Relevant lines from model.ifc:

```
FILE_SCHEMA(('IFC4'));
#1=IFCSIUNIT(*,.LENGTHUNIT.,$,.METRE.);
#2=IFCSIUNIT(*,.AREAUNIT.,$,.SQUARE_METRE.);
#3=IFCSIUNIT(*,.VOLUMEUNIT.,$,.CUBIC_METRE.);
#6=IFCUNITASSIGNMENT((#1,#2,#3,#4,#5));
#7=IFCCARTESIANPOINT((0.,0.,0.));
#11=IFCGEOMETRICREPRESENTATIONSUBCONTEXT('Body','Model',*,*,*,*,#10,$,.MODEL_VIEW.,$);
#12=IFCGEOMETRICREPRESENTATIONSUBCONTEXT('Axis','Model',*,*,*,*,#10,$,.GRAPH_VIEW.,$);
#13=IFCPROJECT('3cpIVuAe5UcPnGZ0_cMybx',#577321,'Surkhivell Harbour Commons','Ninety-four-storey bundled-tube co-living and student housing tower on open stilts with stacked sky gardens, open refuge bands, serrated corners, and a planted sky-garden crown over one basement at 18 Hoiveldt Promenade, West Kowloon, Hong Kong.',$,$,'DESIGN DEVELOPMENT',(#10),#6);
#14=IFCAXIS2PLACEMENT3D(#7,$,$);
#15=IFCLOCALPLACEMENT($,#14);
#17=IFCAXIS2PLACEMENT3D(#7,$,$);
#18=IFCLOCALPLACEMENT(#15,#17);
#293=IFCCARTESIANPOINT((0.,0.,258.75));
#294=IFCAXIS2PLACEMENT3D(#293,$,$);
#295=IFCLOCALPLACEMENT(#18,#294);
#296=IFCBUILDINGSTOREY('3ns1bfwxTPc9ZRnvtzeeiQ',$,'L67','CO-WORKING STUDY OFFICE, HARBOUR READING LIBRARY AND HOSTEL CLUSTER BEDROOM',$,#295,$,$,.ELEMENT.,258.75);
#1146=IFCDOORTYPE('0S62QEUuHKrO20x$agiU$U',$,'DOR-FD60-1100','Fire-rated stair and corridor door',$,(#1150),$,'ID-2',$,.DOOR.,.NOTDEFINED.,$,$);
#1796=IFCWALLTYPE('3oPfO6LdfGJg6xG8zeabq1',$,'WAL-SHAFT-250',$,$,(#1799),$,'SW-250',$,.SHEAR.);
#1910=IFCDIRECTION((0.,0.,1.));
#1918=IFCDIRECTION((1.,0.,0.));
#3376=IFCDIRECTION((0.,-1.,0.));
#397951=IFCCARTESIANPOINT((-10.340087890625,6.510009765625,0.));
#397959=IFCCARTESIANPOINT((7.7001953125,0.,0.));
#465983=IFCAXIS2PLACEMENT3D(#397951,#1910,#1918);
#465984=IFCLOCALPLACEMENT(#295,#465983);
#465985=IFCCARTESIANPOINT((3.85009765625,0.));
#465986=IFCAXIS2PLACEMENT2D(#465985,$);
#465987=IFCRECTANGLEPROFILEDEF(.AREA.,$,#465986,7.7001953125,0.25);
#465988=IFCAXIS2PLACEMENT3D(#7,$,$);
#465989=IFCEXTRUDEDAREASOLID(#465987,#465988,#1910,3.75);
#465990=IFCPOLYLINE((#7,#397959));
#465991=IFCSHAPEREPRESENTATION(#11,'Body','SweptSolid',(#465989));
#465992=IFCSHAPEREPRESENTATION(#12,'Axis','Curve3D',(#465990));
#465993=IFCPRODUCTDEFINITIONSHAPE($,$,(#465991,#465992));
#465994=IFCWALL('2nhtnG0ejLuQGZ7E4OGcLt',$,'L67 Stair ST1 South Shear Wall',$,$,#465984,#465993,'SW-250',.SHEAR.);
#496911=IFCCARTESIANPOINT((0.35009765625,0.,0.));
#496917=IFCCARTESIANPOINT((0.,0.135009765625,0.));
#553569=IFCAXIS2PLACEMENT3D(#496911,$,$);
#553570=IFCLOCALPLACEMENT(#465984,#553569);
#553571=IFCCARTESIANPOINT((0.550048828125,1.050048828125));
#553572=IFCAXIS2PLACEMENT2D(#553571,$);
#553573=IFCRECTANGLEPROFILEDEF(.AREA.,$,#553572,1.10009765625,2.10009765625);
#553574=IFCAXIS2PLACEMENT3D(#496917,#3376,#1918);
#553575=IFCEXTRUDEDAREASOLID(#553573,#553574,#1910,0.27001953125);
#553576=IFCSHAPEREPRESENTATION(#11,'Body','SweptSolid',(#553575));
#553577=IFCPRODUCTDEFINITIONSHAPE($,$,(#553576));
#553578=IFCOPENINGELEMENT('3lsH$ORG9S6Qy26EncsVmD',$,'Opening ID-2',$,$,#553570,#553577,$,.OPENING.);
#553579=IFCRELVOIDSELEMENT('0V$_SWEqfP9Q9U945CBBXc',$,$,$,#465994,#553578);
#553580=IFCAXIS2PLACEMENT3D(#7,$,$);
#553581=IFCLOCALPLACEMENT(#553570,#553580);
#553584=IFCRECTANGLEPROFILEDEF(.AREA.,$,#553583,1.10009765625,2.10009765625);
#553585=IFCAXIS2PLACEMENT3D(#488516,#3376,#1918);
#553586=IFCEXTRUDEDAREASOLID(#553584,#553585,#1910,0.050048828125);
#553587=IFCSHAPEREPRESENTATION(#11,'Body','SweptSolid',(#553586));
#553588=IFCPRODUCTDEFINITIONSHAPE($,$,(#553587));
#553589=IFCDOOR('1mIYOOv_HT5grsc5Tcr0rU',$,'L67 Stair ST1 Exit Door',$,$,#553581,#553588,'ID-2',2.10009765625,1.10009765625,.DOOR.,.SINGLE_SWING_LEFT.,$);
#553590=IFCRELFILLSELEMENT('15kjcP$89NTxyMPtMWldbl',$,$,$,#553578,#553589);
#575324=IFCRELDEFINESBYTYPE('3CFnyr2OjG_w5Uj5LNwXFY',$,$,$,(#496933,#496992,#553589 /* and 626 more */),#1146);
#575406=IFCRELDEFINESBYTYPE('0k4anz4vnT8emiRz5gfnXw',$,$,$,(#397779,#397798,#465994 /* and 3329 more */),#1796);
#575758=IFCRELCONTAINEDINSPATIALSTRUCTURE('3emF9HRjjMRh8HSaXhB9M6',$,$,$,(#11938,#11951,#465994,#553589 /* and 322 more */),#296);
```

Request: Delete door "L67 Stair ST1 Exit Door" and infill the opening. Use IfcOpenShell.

```python
import ifcopenshell
import ifcopenshell.api.feature
import ifcopenshell.api.root
import ifcopenshell.geom
import ifcopenshell.util.shape

model = ifcopenshell.open("model.ifc")
settings = ifcopenshell.geom.settings()


def volume(element):
    """Net volume in cubic metres, openings subtracted."""
    shape = ifcopenshell.geom.create_shape(settings, element)
    return ifcopenshell.util.shape.get_volume(shape.geometry)


door = model.by_guid("1mIYOOv_HT5grsc5Tcr0rU")
opening = door.FillsVoids[0].RelatingOpeningElement
wall = opening.VoidsElements[0].RelatingBuildingElement
before = volume(wall)

ifcopenshell.api.root.remove_product(model, product=door)
ifcopenshell.api.feature.remove_feature(model, feature=opening)

after = volume(wall)

print(f"wall volume {before:.3f} -> {after:.3f} m3")

model.write("model_edited.ifc")
```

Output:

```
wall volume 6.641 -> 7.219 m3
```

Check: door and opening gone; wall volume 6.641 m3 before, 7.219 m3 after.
